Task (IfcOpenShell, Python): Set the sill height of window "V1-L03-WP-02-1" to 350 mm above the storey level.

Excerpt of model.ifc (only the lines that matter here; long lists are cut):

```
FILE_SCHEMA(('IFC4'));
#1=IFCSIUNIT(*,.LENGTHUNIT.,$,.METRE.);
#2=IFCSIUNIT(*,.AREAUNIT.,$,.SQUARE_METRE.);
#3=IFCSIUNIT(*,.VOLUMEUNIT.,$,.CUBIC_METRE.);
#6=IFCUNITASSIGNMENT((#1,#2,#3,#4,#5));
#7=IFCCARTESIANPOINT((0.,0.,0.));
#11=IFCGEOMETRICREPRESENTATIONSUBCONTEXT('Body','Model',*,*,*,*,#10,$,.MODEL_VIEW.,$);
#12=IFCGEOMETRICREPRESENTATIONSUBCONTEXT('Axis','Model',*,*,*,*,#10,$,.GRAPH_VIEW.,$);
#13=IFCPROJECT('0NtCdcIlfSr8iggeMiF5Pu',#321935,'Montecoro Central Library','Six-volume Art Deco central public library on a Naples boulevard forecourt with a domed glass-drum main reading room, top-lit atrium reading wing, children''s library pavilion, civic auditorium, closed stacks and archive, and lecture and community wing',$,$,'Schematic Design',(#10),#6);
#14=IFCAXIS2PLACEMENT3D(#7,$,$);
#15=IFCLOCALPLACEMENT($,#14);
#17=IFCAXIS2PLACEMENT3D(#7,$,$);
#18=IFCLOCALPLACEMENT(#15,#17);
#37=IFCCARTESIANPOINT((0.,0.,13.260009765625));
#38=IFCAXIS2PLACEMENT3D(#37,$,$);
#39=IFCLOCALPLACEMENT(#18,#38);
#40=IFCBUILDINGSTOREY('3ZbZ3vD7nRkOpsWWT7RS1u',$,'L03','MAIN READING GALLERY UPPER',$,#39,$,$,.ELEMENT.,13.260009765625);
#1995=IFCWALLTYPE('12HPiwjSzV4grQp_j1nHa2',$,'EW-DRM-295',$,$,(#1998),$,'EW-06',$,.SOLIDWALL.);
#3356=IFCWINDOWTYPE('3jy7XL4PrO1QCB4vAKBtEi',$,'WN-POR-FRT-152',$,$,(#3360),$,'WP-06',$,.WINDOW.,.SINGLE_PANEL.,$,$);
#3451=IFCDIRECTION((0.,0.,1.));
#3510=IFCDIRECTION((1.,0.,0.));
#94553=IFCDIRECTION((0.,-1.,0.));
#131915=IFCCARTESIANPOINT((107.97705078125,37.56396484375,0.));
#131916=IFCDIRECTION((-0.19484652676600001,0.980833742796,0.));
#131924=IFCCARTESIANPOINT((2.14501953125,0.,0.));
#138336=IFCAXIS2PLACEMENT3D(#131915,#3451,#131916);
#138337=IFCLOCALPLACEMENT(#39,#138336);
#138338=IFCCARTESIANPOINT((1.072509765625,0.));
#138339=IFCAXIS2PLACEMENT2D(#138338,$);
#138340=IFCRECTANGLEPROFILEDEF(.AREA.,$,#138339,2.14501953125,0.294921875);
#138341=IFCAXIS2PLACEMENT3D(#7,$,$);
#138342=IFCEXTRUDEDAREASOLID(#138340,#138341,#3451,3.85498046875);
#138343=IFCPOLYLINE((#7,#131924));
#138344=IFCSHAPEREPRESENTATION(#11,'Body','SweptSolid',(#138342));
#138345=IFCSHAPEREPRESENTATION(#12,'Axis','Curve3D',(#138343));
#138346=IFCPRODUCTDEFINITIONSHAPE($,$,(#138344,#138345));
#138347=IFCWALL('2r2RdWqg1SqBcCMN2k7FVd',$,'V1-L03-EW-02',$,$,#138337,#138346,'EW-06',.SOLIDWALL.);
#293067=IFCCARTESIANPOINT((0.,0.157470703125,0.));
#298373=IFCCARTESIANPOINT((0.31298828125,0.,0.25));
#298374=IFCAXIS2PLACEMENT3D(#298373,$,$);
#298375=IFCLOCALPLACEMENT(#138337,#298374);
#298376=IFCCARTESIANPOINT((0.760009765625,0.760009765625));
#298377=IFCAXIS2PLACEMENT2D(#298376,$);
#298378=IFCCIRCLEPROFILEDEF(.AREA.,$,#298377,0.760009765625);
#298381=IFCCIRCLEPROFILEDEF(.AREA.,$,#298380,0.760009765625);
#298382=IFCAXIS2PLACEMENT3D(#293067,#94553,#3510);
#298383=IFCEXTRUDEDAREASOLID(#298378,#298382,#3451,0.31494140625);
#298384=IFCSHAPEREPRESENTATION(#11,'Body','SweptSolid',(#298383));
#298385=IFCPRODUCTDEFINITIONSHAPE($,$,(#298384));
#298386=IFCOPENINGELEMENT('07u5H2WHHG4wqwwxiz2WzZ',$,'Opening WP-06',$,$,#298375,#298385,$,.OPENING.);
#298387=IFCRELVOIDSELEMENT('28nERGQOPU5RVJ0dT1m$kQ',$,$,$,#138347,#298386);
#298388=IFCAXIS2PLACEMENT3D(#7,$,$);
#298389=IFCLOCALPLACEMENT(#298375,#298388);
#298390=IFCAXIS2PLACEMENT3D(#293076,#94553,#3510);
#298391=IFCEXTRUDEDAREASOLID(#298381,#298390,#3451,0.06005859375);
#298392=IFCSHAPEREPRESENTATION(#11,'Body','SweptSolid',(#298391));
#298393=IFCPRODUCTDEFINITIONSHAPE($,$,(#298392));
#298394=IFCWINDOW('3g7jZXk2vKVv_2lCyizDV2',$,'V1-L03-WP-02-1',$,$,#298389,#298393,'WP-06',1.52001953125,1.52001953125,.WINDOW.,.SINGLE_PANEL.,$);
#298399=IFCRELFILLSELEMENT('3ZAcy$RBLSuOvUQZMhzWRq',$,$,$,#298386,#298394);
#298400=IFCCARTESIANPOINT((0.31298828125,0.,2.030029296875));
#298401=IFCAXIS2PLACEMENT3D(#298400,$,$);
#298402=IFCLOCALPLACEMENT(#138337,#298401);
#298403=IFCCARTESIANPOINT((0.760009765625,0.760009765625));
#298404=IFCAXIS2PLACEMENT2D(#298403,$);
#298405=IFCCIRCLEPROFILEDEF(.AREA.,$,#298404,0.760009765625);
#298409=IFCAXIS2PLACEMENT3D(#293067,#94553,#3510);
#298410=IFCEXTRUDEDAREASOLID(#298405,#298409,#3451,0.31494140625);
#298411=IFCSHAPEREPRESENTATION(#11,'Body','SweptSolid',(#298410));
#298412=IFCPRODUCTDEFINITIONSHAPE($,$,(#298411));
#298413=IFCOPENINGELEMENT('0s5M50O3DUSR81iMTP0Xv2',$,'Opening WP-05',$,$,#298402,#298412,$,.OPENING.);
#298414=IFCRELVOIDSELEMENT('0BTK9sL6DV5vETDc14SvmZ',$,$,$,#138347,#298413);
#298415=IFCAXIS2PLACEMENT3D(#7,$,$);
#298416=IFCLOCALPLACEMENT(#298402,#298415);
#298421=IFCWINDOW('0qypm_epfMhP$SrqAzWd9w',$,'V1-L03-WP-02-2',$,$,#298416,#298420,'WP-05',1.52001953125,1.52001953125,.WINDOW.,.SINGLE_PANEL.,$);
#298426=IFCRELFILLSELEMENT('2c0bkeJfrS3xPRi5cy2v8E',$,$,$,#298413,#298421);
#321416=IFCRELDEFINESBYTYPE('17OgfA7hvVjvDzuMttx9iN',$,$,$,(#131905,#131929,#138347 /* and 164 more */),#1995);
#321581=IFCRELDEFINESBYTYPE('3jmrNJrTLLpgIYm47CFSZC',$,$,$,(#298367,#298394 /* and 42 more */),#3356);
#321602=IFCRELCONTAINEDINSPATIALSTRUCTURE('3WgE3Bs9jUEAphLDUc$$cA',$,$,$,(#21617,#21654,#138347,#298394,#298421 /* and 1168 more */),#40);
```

```python
import numpy as np
import ifcopenshell
import ifcopenshell.api.geometry
import ifcopenshell.geom
import ifcopenshell.util.element
import ifcopenshell.util.placement
import ifcopenshell.util.shape
import ifcopenshell.util.unit

model = ifcopenshell.open("model.ifc")
unit_scale = ifcopenshell.util.unit.calculate_unit_scale(model)

window = model.by_guid("3g7jZXk2vKVv_2lCyizDV2")
opening = window.FillsVoids[0].RelatingOpeningElement
storey = ifcopenshell.util.element.get_container(window, ifc_class="IfcBuildingStorey")
level = ifcopenshell.util.placement.get_local_placement(storey.ObjectPlacement)[2, 3]

# The opening's origin need not be at the sill, so measure its lowest point.
shape = ifcopenshell.geom.create_shape(ifcopenshell.geom.settings(), opening)
bottom = ifcopenshell.util.shape.get_shape_bottom_elevation(shape, shape.geometry) / unit_scale
dz = level + 0.35 - bottom

shift = np.array([0.0, 0.0, dz])
# The window is placed relative to its opening, so it follows when the opening moves.
matrix = ifcopenshell.util.placement.get_local_placement(opening.ObjectPlacement)
matrix[:3, 3] += shift
ifcopenshell.api.geometry.edit_object_placement(
    model, product=opening, matrix=matrix, is_si=False, should_transform_children=True
)

print(f"moved by {dz * unit_scale:+.3f} m")

model.write("model_updated.ifc")
```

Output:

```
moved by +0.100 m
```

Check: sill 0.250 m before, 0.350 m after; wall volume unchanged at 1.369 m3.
